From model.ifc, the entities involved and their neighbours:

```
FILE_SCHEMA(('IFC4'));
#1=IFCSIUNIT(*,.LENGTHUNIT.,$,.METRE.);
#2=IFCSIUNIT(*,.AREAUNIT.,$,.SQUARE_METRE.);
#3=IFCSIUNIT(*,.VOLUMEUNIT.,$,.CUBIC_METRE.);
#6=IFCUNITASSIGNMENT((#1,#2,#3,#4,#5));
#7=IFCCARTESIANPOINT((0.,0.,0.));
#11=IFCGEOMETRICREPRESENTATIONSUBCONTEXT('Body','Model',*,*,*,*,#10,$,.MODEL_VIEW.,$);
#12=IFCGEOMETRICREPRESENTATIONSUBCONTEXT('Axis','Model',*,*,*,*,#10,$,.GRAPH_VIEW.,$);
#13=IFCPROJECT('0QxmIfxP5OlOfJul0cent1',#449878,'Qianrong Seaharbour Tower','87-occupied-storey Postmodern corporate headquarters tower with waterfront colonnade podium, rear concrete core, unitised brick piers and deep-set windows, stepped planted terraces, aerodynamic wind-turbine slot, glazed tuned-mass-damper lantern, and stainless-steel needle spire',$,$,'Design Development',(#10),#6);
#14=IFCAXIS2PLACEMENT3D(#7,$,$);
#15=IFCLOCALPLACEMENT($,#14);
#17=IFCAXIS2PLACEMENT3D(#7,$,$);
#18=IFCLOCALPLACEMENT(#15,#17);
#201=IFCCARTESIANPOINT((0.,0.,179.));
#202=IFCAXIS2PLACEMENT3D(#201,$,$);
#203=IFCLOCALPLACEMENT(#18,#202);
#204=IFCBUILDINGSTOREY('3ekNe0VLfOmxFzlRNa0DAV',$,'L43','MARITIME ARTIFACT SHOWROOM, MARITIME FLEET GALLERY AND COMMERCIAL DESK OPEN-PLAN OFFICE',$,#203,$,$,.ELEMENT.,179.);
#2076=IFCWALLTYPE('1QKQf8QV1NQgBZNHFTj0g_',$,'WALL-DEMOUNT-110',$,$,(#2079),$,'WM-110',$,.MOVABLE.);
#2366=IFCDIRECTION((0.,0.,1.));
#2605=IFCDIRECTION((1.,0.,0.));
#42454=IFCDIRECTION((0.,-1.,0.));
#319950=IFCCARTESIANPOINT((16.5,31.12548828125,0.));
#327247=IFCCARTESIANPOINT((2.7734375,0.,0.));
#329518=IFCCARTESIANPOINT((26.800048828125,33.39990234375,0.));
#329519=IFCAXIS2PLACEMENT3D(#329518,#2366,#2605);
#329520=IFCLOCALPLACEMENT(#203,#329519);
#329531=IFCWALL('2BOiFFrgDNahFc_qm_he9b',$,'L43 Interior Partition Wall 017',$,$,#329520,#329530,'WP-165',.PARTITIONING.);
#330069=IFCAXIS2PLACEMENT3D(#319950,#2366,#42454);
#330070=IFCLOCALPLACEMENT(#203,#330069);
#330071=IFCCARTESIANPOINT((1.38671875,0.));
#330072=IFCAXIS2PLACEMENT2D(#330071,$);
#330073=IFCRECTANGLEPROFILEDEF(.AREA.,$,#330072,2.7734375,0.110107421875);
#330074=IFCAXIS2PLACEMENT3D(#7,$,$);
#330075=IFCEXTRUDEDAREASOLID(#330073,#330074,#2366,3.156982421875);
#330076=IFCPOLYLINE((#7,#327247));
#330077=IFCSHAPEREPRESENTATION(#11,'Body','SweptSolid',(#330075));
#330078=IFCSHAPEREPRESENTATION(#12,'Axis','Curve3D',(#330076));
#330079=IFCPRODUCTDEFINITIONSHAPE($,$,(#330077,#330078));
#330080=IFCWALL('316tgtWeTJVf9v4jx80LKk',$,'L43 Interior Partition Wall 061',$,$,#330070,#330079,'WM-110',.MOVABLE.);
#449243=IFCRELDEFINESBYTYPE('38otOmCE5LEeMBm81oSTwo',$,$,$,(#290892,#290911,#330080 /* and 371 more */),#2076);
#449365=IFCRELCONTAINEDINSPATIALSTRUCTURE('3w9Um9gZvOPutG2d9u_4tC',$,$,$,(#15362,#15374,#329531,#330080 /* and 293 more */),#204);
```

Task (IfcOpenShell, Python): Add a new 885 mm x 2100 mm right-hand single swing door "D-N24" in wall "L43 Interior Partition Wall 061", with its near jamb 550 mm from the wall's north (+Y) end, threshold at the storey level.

```python
import numpy as np
import ifcopenshell
import ifcopenshell.api.feature
import ifcopenshell.api.geometry
import ifcopenshell.api.root
import ifcopenshell.api.spatial
import ifcopenshell.geom
import ifcopenshell.util.element
import ifcopenshell.util.placement
import ifcopenshell.util.representation
import ifcopenshell.util.shape
import ifcopenshell.util.unit

model = ifcopenshell.open("model.ifc")
unit_scale = ifcopenshell.util.unit.calculate_unit_scale(model)
settings = ifcopenshell.geom.settings()


def volume(element):
    """Net volume in cubic metres, openings subtracted."""
    shape = ifcopenshell.geom.create_shape(settings, element)
    return ifcopenshell.util.shape.get_volume(shape.geometry)


wall = model.by_guid("316tgtWeTJVf9v4jx80LKk")
storey = ifcopenshell.util.element.get_container(wall, ifc_class="IfcBuildingStorey")
context = ifcopenshell.util.representation.get_context(model, "Model", "Body", "MODEL_VIEW")
before = volume(wall)

width, height, from_end, sill = 0.885, 2.1, 0.55, 0.0  # metres

# The wall runs along its own X axis, and the end named is its -X end.
wall_shape = ifcopenshell.geom.create_shape(settings, wall)
x, y, z = ifcopenshell.util.shape.get_vertices(wall_shape.geometry).T
start = x.min() + from_end
face, thickness = float(y.min()), float(y.max() - y.min())
wall_matrix = ifcopenshell.util.placement.get_local_placement(wall.ObjectPlacement)
level = ifcopenshell.util.placement.get_local_placement(storey.ObjectPlacement)[2, 3]


def in_wall(x, y):
    """Placement at x, y metres in the wall's axes, at sill height."""
    matrix = wall_matrix.copy()
    matrix[:, 3] = wall_matrix @ np.array([x / unit_scale, y / unit_scale, 0.0, 1.0])
    matrix[2, 3] = level + sill / unit_scale
    return matrix


# Opening: a box that overshoots both wall faces by 50 mm.
opening = ifcopenshell.api.root.create_entity(model, ifc_class="IfcOpeningElement", predefined_type="OPENING")
box = ifcopenshell.api.geometry.add_wall_representation(
    model, context=context, length=width, height=height, thickness=thickness + 0.1
)
ifcopenshell.api.geometry.assign_representation(model, product=opening, representation=box)
ifcopenshell.api.geometry.edit_object_placement(model, product=opening, matrix=in_wall(start, face - 0.05), is_si=False)
ifcopenshell.api.feature.add_feature(model, feature=opening, element=wall)

door = ifcopenshell.api.root.create_entity(model, ifc_class="IfcDoor", name="D-N24", predefined_type="DOOR")
door.OverallWidth, door.OverallHeight = width / unit_scale, height / unit_scale
door.OperationType = "SINGLE_SWING_RIGHT"
body = ifcopenshell.api.geometry.add_door_representation(
    model,
    context=context,
    overall_width=door.OverallWidth,
    overall_height=door.OverallHeight,
    operation_type="SINGLE_SWING_RIGHT",
    lining_properties={"LiningDepth": thickness / unit_scale, "ThresholdDepth": thickness / unit_scale},
)
ifcopenshell.api.geometry.assign_representation(model, product=door, representation=body)
ifcopenshell.api.spatial.assign_container(model, products=[door], relating_structure=storey)
ifcopenshell.api.feature.add_filling(model, opening=opening, element=door)

# The lining spans the wall, so the door starts at the wall face.
ifcopenshell.api.geometry.edit_object_placement(model, product=door, matrix=in_wall(start, face), is_si=False)

after = volume(wall)

print(f"wall volume {before:.3f} -> {after:.3f} m3")

model.write("model-out.ifc")
```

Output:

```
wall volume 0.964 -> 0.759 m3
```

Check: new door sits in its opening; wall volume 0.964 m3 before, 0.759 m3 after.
